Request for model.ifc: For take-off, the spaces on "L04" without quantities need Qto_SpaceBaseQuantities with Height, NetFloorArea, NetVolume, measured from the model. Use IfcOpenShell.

First a look at what the model holds.

```python
import ifcopenshell
import ifcopenshell.util.element
import ifcopenshell.util.unit

model = ifcopenshell.open("model.ifc")
print(model.schema)
for unit_type in ("LENGTHUNIT", "AREAUNIT", "VOLUMEUNIT"):
    print(unit_type, ifcopenshell.util.unit.calculate_unit_scale(model, unit_type))
storey = next(s for s in model.by_type("IfcBuildingStorey") if s.Name == "L04")
spaces = [e for e in ifcopenshell.util.element.get_decomposition(storey) if e.is_a("IfcSpace")]
for e in sorted(spaces, key=lambda e: e.id()):
    print(e.id(), e.is_a(), e.Name, list(ifcopenshell.util.element.get_psets(e, qtos_only=True)), sep=" | ")
```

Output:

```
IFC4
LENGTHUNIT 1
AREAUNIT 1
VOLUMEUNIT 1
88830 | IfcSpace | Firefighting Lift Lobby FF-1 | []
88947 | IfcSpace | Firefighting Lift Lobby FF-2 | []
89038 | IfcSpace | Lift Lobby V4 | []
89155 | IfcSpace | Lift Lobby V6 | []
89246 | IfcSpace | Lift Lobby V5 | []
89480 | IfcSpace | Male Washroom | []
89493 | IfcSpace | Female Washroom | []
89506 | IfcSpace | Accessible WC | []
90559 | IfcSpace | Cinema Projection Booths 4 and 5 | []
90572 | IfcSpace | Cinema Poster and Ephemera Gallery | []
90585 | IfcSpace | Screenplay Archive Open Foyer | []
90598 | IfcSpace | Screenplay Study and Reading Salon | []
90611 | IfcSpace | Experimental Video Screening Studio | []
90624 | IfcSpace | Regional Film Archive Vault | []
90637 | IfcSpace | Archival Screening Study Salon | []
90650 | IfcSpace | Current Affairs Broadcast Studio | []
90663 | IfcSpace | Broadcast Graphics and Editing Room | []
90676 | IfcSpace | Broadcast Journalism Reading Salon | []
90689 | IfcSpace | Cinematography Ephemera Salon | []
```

```python
import ifcopenshell
import ifcopenshell.api.pset
import ifcopenshell.geom
import ifcopenshell.util.element
import ifcopenshell.util.shape
import ifcopenshell.util.unit

model = ifcopenshell.open("model.ifc")
unit_scale = ifcopenshell.util.unit.calculate_unit_scale(model)
area_scale = ifcopenshell.util.unit.calculate_unit_scale(model, "AREAUNIT")
volume_scale = ifcopenshell.util.unit.calculate_unit_scale(model, "VOLUMEUNIT")
settings = ifcopenshell.geom.settings()

storey = next(s for s in model.by_type("IfcBuildingStorey") if s.Name == "L04")
spaces = [e for e in ifcopenshell.util.element.get_decomposition(storey) if e.is_a("IfcSpace")]

for e in sorted(spaces, key=lambda e: e.id()):
    if ifcopenshell.util.element.get_psets(e, qtos_only=True, should_inherit=False):
        continue
    # Geometry comes back in metres, in the element's own axes.
    shape = ifcopenshell.geom.create_shape(settings, e)
    values = {
        "Height": ifcopenshell.util.shape.get_z(shape.geometry) / unit_scale,
        "NetFloorArea": ifcopenshell.util.shape.get_footprint_area(shape.geometry) / area_scale,
        "NetVolume": ifcopenshell.util.shape.get_volume(shape.geometry) / volume_scale,
    }
    qto = ifcopenshell.api.pset.add_qto(model, product=e, name="Qto_SpaceBaseQuantities")
    ifcopenshell.api.pset.edit_qto(model, qto=qto, properties=values)
    print(e.id(), {k: round(v, 3) for k, v in values.items()})

model.write("model_edited.ifc")
```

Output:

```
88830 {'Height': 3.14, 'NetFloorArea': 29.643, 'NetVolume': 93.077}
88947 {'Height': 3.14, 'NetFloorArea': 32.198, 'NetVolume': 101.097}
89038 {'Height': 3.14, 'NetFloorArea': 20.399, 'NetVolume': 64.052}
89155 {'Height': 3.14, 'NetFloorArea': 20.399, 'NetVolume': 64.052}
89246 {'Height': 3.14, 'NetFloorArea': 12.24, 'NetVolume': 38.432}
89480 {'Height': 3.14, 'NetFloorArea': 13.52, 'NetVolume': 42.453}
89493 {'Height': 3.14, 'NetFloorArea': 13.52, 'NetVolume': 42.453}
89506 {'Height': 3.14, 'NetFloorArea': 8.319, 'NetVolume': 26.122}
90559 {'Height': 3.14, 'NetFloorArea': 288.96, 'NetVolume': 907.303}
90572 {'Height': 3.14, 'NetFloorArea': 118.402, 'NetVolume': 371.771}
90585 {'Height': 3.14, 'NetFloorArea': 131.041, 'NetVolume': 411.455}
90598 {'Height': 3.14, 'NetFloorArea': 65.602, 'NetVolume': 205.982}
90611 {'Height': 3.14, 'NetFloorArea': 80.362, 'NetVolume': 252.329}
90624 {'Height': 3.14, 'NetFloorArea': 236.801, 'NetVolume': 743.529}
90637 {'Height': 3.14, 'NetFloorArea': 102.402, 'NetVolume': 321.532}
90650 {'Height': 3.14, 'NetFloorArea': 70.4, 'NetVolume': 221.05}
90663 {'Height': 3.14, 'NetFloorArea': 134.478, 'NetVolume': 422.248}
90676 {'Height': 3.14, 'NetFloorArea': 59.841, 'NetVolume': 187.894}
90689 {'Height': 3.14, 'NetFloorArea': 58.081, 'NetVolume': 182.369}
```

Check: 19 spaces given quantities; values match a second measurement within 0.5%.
